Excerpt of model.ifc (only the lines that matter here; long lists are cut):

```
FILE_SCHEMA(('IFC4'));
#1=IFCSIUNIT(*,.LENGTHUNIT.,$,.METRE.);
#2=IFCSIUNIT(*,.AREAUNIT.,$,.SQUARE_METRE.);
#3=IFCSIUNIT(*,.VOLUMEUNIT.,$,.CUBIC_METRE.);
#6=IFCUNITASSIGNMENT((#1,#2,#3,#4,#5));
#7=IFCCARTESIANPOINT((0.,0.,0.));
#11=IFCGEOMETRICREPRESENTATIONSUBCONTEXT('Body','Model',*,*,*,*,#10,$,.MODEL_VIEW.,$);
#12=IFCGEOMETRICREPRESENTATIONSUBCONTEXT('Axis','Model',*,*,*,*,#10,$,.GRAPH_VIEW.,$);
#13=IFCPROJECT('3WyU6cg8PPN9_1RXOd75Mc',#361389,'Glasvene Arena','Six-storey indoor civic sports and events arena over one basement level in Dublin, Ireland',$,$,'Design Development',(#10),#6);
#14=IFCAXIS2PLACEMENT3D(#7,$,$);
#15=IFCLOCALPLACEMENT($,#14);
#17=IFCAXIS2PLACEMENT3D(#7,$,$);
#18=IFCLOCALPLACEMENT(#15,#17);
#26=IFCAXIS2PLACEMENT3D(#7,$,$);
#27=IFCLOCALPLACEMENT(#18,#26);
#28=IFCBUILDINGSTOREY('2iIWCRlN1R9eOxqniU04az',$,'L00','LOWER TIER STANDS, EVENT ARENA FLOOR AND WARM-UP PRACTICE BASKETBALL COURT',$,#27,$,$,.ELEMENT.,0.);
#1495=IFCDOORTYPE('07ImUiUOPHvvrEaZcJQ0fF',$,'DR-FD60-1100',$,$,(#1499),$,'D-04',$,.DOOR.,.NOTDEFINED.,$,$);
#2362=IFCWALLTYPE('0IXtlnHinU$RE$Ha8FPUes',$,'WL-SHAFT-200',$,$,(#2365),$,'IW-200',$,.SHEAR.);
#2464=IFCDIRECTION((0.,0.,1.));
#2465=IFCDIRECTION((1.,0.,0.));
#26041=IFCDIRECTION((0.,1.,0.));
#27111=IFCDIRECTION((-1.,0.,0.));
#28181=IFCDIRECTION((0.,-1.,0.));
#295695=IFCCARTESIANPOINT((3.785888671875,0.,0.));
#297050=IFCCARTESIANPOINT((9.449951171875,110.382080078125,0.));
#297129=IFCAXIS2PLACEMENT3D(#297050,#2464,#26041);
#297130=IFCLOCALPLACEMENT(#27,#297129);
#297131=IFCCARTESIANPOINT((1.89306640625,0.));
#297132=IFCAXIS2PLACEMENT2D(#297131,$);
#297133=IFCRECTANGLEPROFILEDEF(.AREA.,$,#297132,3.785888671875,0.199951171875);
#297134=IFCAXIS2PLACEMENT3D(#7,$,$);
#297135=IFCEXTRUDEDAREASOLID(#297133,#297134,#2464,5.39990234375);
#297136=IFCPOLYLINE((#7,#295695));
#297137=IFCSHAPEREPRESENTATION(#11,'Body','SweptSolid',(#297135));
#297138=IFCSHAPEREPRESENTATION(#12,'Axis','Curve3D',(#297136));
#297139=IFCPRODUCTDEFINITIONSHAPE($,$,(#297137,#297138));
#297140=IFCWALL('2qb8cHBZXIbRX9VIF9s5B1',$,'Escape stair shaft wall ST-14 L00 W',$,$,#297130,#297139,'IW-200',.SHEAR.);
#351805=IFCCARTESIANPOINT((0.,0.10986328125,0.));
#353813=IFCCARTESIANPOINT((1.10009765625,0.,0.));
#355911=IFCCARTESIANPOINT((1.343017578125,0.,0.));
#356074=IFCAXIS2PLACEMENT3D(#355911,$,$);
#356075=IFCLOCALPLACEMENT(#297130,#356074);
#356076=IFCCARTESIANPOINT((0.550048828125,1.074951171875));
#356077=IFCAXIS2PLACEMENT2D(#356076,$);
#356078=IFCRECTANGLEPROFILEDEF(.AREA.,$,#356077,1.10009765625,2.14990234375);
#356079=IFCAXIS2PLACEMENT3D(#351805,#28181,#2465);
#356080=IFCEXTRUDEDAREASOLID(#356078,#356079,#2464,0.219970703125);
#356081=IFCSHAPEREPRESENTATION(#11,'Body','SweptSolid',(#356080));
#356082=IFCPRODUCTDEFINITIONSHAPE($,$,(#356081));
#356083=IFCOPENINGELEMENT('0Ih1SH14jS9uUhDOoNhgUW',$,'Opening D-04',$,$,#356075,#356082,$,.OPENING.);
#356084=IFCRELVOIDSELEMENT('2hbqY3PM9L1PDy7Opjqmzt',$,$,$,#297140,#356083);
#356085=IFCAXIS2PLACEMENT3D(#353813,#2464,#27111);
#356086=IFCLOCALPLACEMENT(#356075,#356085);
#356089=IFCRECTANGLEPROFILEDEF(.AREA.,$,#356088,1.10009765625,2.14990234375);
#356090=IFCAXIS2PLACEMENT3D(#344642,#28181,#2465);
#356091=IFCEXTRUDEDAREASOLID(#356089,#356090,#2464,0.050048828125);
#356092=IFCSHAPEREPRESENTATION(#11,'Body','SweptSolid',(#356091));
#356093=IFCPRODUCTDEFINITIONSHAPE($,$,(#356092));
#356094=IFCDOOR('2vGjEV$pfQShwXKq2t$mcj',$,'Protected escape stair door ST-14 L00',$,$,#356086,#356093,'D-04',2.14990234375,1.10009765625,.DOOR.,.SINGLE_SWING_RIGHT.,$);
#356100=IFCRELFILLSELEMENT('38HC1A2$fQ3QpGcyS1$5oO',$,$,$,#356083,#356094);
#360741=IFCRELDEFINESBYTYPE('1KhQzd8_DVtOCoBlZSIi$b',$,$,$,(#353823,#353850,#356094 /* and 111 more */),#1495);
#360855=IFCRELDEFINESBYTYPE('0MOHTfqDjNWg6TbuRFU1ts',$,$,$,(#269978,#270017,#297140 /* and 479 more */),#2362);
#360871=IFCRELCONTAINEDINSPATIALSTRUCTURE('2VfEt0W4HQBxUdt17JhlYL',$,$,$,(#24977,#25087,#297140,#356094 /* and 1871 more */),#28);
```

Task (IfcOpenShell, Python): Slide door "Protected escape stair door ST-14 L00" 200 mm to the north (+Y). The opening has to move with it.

```python
import ifcopenshell
import ifcopenshell.api.geometry
import ifcopenshell.util.placement
import ifcopenshell.util.unit

model = ifcopenshell.open("model.ifc")
unit_scale = ifcopenshell.util.unit.calculate_unit_scale(model)

door = model.by_guid("2vGjEV$pfQShwXKq2t$mcj")
opening = door.FillsVoids[0].RelatingOpeningElement
wall = opening.VoidsElements[0].RelatingBuildingElement

wall_matrix = ifcopenshell.util.placement.get_local_placement(wall.ObjectPlacement)
shift = wall_matrix[:3, 0] * 0.2 / unit_scale
before = ifcopenshell.util.placement.get_local_placement(door.ObjectPlacement)[:3, 3].copy()

# The door is placed relative to its opening, so it follows when the opening moves.
matrix = ifcopenshell.util.placement.get_local_placement(opening.ObjectPlacement)
matrix[:3, 3] += shift
ifcopenshell.api.geometry.edit_object_placement(
    model, product=opening, matrix=matrix, is_si=False, should_transform_children=True
)

after = ifcopenshell.util.placement.get_local_placement(door.ObjectPlacement)[:3, 3]
print("door moved by", (after - before).round(3) + 0.0)

model.write("model_updated.ifc")
```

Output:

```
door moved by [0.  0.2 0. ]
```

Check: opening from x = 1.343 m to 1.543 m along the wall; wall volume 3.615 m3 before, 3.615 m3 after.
